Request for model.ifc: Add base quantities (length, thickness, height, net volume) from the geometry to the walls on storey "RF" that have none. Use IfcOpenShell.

First a look at what the model holds.

```python
import ifcopenshell
import ifcopenshell.util.element
import ifcopenshell.util.unit

model = ifcopenshell.open("model.ifc")
print(model.schema)
for unit_type in ("LENGTHUNIT", "AREAUNIT", "VOLUMEUNIT"):
    print(unit_type, ifcopenshell.util.unit.calculate_unit_scale(model, unit_type))
storey = next(s for s in model.by_type("IfcBuildingStorey") if s.Name == "RF")
walls = [e for e in ifcopenshell.util.element.get_decomposition(storey) if e.is_a("IfcWall")]
for e in sorted(walls, key=lambda e: e.id()):
    print(e.id(), e.is_a(), e.Name, list(ifcopenshell.util.element.get_psets(e, qtos_only=True)), sep=" | ")
```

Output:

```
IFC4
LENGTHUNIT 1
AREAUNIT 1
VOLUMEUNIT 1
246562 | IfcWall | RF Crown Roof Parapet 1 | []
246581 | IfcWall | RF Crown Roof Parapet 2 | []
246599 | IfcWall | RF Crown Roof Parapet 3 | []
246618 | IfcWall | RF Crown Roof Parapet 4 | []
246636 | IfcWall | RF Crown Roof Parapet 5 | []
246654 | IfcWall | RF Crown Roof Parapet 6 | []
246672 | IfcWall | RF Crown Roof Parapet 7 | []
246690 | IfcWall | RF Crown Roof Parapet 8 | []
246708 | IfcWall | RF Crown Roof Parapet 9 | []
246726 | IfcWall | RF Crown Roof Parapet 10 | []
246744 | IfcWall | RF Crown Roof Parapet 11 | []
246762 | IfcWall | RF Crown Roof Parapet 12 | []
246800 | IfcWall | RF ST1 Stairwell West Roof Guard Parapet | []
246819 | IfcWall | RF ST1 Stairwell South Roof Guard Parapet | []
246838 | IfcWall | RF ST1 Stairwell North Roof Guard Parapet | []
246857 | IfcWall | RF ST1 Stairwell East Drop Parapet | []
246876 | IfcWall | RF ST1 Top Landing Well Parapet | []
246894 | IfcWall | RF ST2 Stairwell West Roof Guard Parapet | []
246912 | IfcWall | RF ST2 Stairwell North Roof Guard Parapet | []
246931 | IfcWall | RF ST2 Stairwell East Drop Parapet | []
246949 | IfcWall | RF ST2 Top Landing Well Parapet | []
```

```python
import ifcopenshell
import ifcopenshell.api.pset
import ifcopenshell.geom
import ifcopenshell.util.element
import ifcopenshell.util.shape
import ifcopenshell.util.unit

model = ifcopenshell.open("model.ifc")
unit_scale = ifcopenshell.util.unit.calculate_unit_scale(model)
volume_scale = ifcopenshell.util.unit.calculate_unit_scale(model, "VOLUMEUNIT")
settings = ifcopenshell.geom.settings()

storey = next(s for s in model.by_type("IfcBuildingStorey") if s.Name == "RF")
walls = [e for e in ifcopenshell.util.element.get_decomposition(storey) if e.is_a("IfcWall")]

for e in sorted(walls, key=lambda e: e.id()):
    if ifcopenshell.util.element.get_psets(e, qtos_only=True, should_inherit=False):
        continue
    # Geometry comes back in metres, in the element's own axes.
    shape = ifcopenshell.geom.create_shape(settings, e)
    values = {
        "Length": ifcopenshell.util.shape.get_x(shape.geometry) / unit_scale,
        "Width": ifcopenshell.util.shape.get_y(shape.geometry) / unit_scale,
        "Height": ifcopenshell.util.shape.get_z(shape.geometry) / unit_scale,
        "NetVolume": ifcopenshell.util.shape.get_volume(shape.geometry) / volume_scale,
    }
    qto = ifcopenshell.api.pset.add_qto(model, product=e, name="Qto_WallBaseQuantities")
    ifcopenshell.api.pset.edit_qto(model, qto=qto, properties=values)
    print(e.id(), {k: round(v, 3) for k, v in values.items()})

model.write("model_updated.ifc")
```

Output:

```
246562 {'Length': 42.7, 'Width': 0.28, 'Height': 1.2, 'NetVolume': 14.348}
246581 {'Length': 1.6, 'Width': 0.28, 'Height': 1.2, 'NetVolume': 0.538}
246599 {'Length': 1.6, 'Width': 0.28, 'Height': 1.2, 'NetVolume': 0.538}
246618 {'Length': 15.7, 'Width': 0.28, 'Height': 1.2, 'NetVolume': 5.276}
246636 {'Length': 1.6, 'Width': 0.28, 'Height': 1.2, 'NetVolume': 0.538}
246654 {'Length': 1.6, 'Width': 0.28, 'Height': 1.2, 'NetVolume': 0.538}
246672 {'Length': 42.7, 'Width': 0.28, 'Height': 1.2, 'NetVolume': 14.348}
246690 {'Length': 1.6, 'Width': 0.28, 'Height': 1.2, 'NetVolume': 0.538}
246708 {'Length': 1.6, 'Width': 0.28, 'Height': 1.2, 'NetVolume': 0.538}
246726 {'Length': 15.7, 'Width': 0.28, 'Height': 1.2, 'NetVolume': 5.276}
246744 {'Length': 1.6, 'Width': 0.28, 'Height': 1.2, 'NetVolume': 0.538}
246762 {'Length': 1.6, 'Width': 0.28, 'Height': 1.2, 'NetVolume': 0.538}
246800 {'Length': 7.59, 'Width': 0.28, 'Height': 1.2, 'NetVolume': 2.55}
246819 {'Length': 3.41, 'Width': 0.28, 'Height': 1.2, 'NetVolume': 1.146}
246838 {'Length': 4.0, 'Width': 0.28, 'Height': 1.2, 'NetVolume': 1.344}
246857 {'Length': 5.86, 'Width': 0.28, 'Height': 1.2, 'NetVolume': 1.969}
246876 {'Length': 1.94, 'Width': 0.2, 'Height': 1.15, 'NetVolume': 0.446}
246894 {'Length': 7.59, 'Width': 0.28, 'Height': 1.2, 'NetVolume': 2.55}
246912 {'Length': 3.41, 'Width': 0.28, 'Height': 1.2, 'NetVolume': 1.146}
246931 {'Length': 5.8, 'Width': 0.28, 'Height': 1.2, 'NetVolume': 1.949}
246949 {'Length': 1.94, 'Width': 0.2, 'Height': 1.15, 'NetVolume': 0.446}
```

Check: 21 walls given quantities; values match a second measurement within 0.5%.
